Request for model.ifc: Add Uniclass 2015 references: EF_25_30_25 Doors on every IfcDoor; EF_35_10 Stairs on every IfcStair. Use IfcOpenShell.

First a look at what the model holds.

```python
import ifcopenshell

model = ifcopenshell.open("model.ifc")
print(model.schema)
print("classifications:", [c.Name for c in model.by_type("IfcClassification")])
for ifc_class in ("IfcDoor", "IfcRoof", "IfcStair", "IfcWall", "IfcWindow"):
    print(ifc_class, len(model.by_type(ifc_class)))
```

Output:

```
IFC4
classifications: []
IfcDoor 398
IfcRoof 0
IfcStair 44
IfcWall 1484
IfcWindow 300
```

```python
import ifcopenshell
import ifcopenshell.api.classification

model = ifcopenshell.open("model.ifc")

system = ifcopenshell.api.classification.add_classification(model, classification="Uniclass 2015")

codes = {
    "IfcDoor": ("EF_25_30_25", "Doors"),
    "IfcStair": ("EF_35_10", "Stairs"),
}
for ifc_class, (code, name) in codes.items():
    products = model.by_type(ifc_class)
    ifcopenshell.api.classification.add_reference(
        model, products=products, classification=system, identification=code, name=name
    )
    print(code, len(products))

model.write("model_updated.ifc")
```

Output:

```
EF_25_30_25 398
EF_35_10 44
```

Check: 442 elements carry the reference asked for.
